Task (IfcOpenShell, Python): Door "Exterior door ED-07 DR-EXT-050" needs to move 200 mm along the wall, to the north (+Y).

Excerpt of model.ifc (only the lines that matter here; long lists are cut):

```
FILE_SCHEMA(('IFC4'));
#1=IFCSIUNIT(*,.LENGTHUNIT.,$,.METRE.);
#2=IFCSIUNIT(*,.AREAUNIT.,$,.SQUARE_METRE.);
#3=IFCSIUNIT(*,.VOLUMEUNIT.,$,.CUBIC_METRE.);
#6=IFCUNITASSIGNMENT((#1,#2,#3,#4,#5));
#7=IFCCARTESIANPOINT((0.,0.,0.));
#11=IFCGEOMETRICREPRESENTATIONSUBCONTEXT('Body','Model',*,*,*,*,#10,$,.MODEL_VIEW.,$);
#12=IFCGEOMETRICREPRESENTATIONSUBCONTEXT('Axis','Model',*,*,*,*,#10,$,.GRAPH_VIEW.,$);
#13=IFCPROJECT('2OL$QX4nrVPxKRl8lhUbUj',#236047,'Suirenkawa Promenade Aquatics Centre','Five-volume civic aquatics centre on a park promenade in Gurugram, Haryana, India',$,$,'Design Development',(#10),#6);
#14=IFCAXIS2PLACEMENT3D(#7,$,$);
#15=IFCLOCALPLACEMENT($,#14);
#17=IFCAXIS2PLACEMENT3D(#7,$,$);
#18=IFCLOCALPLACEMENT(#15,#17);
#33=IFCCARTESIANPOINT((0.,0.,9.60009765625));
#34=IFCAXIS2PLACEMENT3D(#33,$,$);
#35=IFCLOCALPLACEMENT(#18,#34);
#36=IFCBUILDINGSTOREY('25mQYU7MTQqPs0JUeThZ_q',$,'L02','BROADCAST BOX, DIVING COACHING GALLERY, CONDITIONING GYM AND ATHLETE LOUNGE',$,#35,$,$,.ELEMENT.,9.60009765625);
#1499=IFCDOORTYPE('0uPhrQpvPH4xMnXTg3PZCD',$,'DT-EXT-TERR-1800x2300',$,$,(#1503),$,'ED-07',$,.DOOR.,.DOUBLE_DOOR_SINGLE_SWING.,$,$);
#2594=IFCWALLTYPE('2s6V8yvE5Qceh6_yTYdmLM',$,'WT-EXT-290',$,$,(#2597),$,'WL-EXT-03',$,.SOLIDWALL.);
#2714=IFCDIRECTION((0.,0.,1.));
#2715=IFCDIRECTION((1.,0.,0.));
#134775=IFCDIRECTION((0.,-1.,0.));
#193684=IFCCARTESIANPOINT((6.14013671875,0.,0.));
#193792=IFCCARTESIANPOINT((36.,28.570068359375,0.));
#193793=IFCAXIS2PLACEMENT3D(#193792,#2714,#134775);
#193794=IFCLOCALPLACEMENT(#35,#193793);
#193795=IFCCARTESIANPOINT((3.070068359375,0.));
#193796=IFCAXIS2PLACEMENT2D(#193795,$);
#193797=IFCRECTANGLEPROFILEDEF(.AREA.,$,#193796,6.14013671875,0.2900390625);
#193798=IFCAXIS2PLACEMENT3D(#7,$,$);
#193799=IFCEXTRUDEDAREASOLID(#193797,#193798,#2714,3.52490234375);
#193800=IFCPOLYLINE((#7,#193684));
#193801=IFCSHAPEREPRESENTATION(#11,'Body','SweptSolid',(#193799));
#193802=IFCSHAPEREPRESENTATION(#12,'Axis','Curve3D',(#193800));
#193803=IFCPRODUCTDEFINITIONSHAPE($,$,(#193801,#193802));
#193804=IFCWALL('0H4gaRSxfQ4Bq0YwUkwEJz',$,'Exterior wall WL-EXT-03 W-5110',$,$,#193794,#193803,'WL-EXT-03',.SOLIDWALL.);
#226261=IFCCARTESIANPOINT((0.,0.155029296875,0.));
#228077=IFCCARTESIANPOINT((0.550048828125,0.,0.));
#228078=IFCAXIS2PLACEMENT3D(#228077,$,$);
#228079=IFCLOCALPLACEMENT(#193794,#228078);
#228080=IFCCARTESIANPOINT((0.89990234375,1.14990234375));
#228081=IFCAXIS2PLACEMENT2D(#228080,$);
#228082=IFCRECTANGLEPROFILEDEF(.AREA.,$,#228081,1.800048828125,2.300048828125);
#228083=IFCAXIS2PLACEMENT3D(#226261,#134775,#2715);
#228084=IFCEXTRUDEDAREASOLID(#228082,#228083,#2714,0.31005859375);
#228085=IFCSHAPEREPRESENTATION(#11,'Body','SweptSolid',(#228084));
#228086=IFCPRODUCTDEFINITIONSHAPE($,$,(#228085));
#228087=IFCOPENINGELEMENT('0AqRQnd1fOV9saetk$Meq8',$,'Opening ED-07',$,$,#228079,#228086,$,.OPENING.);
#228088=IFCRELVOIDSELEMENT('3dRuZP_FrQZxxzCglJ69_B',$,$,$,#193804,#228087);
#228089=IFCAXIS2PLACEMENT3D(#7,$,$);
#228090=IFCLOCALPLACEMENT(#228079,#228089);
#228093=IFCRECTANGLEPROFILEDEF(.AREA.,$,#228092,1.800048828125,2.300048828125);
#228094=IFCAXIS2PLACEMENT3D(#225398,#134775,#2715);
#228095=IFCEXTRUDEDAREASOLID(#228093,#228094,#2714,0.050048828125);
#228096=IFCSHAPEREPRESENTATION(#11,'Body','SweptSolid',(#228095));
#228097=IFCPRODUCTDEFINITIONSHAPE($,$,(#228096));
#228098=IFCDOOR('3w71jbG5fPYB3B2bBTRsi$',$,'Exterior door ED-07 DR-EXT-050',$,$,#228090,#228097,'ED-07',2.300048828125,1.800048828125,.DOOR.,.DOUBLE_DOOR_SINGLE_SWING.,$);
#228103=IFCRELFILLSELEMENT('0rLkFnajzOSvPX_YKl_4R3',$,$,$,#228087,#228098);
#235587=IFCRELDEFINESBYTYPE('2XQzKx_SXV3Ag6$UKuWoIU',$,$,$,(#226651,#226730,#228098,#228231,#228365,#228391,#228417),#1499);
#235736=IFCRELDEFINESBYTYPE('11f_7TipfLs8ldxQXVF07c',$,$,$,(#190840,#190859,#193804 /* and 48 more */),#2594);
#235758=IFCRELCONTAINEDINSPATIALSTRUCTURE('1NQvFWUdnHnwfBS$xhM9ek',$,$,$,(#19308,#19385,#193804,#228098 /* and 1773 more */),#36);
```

```python
import ifcopenshell
import ifcopenshell.api.geometry
import ifcopenshell.util.placement

model = ifcopenshell.open("model.ifc")

door = model.by_id(228098)
opening = door.FillsVoids[0].RelatingOpeningElement
wall = opening.VoidsElements[0].RelatingBuildingElement

wall_matrix = ifcopenshell.util.placement.get_local_placement(wall.ObjectPlacement)
shift = wall_matrix[:3, 0] * -0.2
before = ifcopenshell.util.placement.get_local_placement(door.ObjectPlacement)[:3, 3].copy()

# The door is placed relative to its opening, so it follows when the opening moves.
matrix = ifcopenshell.util.placement.get_local_placement(opening.ObjectPlacement)
matrix[:3, 3] += shift
ifcopenshell.api.geometry.edit_object_placement(
    model, product=opening, matrix=matrix, is_si=False, should_transform_children=True
)

after = ifcopenshell.util.placement.get_local_placement(door.ObjectPlacement)[:3, 3]
print("door moved by", (after - before).round(3) + 0.0)

model.write("model_updated.ifc")
```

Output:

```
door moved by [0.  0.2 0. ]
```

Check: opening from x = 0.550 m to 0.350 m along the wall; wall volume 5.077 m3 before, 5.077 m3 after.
